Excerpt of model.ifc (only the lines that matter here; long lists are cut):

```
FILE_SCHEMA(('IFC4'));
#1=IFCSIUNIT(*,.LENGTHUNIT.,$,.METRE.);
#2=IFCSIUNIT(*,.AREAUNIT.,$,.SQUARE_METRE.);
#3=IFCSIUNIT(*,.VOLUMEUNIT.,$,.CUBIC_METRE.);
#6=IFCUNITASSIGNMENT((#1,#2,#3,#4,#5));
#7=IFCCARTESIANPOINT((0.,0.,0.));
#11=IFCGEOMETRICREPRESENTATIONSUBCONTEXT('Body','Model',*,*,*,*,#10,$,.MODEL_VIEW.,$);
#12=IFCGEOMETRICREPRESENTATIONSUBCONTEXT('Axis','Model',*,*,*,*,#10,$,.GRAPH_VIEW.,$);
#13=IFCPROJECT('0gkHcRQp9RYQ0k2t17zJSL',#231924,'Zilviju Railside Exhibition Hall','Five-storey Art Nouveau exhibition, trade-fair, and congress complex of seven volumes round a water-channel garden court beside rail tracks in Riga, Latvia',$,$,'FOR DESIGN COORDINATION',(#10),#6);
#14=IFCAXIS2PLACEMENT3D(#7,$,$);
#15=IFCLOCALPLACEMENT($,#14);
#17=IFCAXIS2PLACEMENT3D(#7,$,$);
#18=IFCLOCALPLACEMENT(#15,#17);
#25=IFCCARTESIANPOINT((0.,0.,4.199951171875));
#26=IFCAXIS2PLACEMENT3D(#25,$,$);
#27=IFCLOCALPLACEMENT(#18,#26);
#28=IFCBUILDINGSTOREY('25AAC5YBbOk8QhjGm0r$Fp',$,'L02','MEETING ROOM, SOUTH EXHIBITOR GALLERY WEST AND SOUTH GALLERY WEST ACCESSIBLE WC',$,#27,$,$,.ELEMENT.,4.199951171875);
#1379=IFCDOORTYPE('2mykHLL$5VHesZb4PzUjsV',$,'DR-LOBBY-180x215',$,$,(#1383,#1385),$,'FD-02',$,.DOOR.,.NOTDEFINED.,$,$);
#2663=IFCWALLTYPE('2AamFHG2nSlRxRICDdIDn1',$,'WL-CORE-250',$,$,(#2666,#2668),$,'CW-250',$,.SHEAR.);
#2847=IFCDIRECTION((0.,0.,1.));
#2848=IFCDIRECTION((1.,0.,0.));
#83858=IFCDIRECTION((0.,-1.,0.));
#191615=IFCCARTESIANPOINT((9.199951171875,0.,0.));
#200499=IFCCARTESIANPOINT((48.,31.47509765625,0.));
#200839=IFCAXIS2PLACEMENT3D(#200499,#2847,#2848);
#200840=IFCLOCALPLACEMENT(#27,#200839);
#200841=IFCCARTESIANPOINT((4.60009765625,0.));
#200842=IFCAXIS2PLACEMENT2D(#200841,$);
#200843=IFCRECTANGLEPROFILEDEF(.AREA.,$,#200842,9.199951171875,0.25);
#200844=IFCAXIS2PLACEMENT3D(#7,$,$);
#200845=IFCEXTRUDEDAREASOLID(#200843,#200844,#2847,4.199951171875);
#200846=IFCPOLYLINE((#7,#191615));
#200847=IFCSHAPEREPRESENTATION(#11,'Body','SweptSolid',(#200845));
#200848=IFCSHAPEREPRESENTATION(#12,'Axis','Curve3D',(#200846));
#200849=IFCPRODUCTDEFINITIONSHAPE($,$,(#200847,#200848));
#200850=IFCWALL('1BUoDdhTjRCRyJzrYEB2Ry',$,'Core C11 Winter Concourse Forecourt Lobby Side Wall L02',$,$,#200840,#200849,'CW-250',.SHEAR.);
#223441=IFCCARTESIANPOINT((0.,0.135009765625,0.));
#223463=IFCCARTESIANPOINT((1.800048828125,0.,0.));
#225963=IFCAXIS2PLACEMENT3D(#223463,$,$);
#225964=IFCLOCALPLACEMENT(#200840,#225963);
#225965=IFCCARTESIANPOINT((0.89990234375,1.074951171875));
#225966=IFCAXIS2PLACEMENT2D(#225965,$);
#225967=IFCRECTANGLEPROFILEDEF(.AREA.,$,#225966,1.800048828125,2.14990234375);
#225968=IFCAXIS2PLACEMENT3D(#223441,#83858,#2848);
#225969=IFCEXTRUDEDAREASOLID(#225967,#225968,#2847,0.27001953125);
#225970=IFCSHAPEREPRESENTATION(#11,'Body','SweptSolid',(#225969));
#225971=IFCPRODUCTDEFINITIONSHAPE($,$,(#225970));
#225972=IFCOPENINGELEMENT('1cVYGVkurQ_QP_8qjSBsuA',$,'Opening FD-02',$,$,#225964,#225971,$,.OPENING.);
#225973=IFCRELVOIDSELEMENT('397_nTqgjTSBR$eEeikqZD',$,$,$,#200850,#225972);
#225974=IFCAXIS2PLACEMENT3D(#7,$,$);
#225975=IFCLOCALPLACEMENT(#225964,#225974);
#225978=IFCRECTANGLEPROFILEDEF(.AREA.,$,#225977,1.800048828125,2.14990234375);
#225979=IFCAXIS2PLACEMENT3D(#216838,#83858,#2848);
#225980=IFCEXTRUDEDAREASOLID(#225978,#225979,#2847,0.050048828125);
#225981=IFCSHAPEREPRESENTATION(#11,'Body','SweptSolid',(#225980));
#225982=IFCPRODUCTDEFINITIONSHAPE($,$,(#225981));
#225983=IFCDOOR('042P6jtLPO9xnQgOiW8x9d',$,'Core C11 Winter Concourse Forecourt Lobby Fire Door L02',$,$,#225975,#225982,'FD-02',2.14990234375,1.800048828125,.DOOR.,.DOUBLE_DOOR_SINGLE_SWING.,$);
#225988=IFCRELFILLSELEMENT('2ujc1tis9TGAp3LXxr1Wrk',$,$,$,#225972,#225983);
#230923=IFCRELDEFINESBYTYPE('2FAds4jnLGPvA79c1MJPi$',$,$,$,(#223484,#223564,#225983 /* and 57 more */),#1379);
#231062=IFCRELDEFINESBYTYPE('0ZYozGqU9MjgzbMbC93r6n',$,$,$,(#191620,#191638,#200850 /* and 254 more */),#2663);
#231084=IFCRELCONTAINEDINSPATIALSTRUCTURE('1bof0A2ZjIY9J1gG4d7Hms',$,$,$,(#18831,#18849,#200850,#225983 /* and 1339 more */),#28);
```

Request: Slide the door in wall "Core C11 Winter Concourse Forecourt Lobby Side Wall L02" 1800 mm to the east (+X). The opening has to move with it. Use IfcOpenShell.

```python
import ifcopenshell
import ifcopenshell.api.geometry
import ifcopenshell.util.placement

model = ifcopenshell.open("model.ifc")

door = model.by_guid("042P6jtLPO9xnQgOiW8x9d")
opening = door.FillsVoids[0].RelatingOpeningElement
wall = opening.VoidsElements[0].RelatingBuildingElement

wall_matrix = ifcopenshell.util.placement.get_local_placement(wall.ObjectPlacement)
shift = wall_matrix[:3, 0] * 1.8
before = ifcopenshell.util.placement.get_local_placement(door.ObjectPlacement)[:3, 3].copy()

# The door is placed relative to its opening, so it follows when the opening moves.
matrix = ifcopenshell.util.placement.get_local_placement(opening.ObjectPlacement)
matrix[:3, 3] += shift
ifcopenshell.api.geometry.edit_object_placement(
    model, product=opening, matrix=matrix, is_si=False, should_transform_children=True
)

after = ifcopenshell.util.placement.get_local_placement(door.ObjectPlacement)[:3, 3]
print("door moved by", (after - before).round(3) + 0.0)

model.write("model_v2.ifc")
```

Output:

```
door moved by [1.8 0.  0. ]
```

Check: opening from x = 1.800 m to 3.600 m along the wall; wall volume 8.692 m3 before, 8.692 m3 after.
